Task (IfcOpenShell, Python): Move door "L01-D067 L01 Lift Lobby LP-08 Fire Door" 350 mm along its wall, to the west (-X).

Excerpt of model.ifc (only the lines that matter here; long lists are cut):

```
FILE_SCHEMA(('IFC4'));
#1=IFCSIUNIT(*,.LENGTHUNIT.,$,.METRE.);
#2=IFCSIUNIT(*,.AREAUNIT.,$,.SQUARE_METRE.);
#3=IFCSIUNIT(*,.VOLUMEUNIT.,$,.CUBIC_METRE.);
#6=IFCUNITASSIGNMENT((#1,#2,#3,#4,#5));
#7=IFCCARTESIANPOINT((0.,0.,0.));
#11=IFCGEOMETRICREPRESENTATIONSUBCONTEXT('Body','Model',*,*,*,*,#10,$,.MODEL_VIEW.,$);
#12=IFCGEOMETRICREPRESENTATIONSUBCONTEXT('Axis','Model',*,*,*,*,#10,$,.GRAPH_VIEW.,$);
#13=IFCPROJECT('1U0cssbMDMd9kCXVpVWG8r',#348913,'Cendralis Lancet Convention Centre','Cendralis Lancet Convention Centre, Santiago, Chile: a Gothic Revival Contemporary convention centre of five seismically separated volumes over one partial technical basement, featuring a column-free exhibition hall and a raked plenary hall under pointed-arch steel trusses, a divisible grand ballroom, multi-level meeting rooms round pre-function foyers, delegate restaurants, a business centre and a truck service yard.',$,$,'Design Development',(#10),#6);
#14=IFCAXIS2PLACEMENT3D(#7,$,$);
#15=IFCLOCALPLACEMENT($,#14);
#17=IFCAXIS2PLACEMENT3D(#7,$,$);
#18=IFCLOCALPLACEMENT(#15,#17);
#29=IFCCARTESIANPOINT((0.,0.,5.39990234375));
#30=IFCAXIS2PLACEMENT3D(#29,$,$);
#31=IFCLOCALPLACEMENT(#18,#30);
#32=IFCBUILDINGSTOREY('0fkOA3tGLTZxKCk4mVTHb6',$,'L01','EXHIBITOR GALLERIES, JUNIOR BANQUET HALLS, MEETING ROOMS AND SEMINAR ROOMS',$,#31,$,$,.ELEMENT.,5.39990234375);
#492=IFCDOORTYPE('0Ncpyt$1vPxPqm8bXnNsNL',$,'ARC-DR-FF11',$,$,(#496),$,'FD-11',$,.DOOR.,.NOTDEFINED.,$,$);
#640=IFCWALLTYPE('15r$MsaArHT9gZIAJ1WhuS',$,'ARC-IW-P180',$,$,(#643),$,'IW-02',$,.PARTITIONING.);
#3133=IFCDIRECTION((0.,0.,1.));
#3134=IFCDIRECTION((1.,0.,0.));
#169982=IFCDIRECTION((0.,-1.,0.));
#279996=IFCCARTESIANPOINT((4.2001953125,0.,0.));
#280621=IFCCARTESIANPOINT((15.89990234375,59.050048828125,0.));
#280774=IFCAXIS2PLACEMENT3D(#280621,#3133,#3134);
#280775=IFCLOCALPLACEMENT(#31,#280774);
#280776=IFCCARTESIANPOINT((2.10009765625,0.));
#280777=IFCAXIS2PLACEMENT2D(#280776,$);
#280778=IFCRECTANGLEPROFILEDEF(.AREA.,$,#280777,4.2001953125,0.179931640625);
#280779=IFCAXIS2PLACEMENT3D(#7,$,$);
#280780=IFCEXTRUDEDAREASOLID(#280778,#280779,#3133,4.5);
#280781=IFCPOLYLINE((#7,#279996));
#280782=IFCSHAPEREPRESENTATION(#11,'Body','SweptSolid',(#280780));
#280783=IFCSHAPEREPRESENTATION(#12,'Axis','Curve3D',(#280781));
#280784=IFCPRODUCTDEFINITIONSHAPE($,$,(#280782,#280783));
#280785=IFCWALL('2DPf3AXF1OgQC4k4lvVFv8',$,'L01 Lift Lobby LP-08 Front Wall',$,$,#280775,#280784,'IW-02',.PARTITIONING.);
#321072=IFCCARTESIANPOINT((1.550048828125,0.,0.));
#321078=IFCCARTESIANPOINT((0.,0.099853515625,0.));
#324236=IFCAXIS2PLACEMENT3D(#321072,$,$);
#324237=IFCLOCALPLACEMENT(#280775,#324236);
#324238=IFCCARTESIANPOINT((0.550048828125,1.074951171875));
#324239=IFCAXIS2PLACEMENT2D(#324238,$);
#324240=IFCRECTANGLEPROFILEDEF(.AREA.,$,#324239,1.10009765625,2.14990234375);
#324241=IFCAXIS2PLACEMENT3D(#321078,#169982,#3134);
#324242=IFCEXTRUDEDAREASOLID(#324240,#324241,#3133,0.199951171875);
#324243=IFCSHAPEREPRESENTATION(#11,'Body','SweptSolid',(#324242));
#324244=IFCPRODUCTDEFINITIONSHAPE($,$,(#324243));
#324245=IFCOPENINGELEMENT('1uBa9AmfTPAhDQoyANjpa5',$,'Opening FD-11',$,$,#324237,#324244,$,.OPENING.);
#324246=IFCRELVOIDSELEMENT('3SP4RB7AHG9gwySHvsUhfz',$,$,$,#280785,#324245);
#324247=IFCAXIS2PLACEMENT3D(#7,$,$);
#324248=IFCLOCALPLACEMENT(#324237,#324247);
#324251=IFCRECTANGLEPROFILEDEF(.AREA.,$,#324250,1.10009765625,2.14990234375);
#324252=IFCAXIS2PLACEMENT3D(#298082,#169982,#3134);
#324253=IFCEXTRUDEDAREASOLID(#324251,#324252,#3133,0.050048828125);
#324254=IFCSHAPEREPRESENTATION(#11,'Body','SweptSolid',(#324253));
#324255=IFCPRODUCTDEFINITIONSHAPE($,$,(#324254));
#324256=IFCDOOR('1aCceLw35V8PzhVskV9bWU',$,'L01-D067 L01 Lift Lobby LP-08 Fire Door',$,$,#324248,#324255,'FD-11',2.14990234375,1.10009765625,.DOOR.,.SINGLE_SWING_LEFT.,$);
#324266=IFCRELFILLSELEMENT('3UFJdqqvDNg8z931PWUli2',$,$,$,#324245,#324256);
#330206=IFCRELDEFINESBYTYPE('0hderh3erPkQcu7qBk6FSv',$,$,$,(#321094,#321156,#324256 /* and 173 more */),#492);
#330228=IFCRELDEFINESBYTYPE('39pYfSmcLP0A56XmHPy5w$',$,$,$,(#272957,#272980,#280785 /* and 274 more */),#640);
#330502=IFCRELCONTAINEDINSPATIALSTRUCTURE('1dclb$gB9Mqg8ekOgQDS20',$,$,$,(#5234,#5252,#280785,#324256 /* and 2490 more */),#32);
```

```python
import ifcopenshell
import ifcopenshell.api.geometry
import ifcopenshell.util.placement

model = ifcopenshell.open("model.ifc")

door = model.by_id(324256)
opening = door.FillsVoids[0].RelatingOpeningElement
wall = opening.VoidsElements[0].RelatingBuildingElement

wall_matrix = ifcopenshell.util.placement.get_local_placement(wall.ObjectPlacement)
shift = wall_matrix[:3, 0] * -0.35
before = ifcopenshell.util.placement.get_local_placement(door.ObjectPlacement)[:3, 3].copy()

# The door is placed relative to its opening, so it follows when the opening moves.
matrix = ifcopenshell.util.placement.get_local_placement(opening.ObjectPlacement)
matrix[:3, 3] += shift
ifcopenshell.api.geometry.edit_object_placement(
    model, product=opening, matrix=matrix, is_si=False, should_transform_children=True
)

after = ifcopenshell.util.placement.get_local_placement(door.ObjectPlacement)[:3, 3]
print("door moved by", (after - before).round(3) + 0.0)

model.write("model_rev.ifc")
```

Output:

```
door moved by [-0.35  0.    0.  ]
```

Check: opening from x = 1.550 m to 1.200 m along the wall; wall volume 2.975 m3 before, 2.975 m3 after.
